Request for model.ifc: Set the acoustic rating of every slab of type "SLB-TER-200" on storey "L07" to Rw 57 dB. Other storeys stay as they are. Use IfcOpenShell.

First a look at what the model holds.

```python
import ifcopenshell
import ifcopenshell.util.element

model = ifcopenshell.open("model.ifc")
print(model.schema)
storey = next(s for s in model.by_type("IfcBuildingStorey") if s.Name == "L07")
slabs = [e for e in ifcopenshell.util.element.get_decomposition(storey) if e.is_a("IfcSlab")]
seen = {}
for e in slabs:
    element_type = ifcopenshell.util.element.get_type(e)
    key = (element_type.Name if element_type != e and element_type else None, ifcopenshell.util.element.get_pset(e, "Pset_SlabCommon", "AcousticRating"))
    seen[key] = seen.get(key, 0) + 1
for (name, value), count in sorted(seen.items(), key=str):
    print(count, "x", name, "|", value)
```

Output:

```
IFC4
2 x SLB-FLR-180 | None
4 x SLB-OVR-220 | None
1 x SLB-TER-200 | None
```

```python
import ifcopenshell
import ifcopenshell.api.pset
import ifcopenshell.util.element

model = ifcopenshell.open("model.ifc")

storey = next(s for s in model.by_type("IfcBuildingStorey") if s.Name == "L07")
slabs = [e for e in ifcopenshell.util.element.get_decomposition(storey) if e.is_a("IfcSlab")]

count = 0
for e in slabs:
    element_type = ifcopenshell.util.element.get_type(e)
    if element_type in (None, e) or element_type.Name != "SLB-TER-200":
        continue
    # add_pset returns the element's existing set when there is one.
    pset = ifcopenshell.api.pset.add_pset(model, product=e, name="Pset_SlabCommon")
    ifcopenshell.api.pset.edit_pset(model, pset=pset, properties={"AcousticRating": "Rw 57 dB"})
    count += 1

print(count, "slabs updated")

model.write("model_updated.ifc")
```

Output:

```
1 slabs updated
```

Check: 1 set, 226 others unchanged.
